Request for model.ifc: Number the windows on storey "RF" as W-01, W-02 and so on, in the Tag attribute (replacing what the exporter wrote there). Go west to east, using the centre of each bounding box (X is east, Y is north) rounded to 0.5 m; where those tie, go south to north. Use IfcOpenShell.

First a look at what the model holds.

```python
import ifcopenshell
import ifcopenshell.util.element
import ifcopenshell.util.placement

model = ifcopenshell.open("model.ifc")
print(model.schema)
storey = next(s for s in model.by_type("IfcBuildingStorey") if s.Name == "RF")
windows = [e for e in ifcopenshell.util.element.get_decomposition(storey) if e.is_a("IfcWindow")]
for e in sorted(windows, key=lambda e: e.id()):
    origin = ifcopenshell.util.placement.get_local_placement(e.ObjectPlacement)[:3, 3]
    print(e.id(), e.Tag, e.Name, origin.round(2) + 0.0, sep=" | ")
```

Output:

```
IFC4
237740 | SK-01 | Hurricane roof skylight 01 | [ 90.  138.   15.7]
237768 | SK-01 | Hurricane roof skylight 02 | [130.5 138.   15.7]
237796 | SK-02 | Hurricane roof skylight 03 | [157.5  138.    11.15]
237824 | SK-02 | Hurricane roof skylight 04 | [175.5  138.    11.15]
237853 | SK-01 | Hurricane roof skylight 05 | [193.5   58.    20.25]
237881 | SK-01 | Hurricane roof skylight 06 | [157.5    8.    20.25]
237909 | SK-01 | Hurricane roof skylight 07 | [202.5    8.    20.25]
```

```python
import ifcopenshell
import ifcopenshell.geom
import ifcopenshell.util.element
import ifcopenshell.util.shape

model = ifcopenshell.open("model.ifc")
settings = ifcopenshell.geom.settings()
settings.set("use-world-coords", True)


def centre(element):
    shape = ifcopenshell.geom.create_shape(settings, element)
    return ifcopenshell.util.shape.get_bbox_centroid(shape.geometry)


storey = next(s for s in model.by_type("IfcBuildingStorey") if s.Name == "RF")
windows = [e for e in ifcopenshell.util.element.get_decomposition(storey) if e.is_a("IfcWindow")]

# Insertion points can sit at a corner or the storey origin, so sort by the geometry (in metres).
centres = {e: centre(e) for e in windows}
windows.sort(key=lambda e: (round(centres[e][0] / 0.5), centres[e][1]))

for i, e in enumerate(windows, start=1):
    number = f"W-{i:02d}"
    e.Tag = number
    print(e.id(), number)

model.write("model_updated.ifc")
```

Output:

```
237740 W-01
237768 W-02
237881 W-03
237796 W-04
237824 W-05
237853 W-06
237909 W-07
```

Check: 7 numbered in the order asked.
